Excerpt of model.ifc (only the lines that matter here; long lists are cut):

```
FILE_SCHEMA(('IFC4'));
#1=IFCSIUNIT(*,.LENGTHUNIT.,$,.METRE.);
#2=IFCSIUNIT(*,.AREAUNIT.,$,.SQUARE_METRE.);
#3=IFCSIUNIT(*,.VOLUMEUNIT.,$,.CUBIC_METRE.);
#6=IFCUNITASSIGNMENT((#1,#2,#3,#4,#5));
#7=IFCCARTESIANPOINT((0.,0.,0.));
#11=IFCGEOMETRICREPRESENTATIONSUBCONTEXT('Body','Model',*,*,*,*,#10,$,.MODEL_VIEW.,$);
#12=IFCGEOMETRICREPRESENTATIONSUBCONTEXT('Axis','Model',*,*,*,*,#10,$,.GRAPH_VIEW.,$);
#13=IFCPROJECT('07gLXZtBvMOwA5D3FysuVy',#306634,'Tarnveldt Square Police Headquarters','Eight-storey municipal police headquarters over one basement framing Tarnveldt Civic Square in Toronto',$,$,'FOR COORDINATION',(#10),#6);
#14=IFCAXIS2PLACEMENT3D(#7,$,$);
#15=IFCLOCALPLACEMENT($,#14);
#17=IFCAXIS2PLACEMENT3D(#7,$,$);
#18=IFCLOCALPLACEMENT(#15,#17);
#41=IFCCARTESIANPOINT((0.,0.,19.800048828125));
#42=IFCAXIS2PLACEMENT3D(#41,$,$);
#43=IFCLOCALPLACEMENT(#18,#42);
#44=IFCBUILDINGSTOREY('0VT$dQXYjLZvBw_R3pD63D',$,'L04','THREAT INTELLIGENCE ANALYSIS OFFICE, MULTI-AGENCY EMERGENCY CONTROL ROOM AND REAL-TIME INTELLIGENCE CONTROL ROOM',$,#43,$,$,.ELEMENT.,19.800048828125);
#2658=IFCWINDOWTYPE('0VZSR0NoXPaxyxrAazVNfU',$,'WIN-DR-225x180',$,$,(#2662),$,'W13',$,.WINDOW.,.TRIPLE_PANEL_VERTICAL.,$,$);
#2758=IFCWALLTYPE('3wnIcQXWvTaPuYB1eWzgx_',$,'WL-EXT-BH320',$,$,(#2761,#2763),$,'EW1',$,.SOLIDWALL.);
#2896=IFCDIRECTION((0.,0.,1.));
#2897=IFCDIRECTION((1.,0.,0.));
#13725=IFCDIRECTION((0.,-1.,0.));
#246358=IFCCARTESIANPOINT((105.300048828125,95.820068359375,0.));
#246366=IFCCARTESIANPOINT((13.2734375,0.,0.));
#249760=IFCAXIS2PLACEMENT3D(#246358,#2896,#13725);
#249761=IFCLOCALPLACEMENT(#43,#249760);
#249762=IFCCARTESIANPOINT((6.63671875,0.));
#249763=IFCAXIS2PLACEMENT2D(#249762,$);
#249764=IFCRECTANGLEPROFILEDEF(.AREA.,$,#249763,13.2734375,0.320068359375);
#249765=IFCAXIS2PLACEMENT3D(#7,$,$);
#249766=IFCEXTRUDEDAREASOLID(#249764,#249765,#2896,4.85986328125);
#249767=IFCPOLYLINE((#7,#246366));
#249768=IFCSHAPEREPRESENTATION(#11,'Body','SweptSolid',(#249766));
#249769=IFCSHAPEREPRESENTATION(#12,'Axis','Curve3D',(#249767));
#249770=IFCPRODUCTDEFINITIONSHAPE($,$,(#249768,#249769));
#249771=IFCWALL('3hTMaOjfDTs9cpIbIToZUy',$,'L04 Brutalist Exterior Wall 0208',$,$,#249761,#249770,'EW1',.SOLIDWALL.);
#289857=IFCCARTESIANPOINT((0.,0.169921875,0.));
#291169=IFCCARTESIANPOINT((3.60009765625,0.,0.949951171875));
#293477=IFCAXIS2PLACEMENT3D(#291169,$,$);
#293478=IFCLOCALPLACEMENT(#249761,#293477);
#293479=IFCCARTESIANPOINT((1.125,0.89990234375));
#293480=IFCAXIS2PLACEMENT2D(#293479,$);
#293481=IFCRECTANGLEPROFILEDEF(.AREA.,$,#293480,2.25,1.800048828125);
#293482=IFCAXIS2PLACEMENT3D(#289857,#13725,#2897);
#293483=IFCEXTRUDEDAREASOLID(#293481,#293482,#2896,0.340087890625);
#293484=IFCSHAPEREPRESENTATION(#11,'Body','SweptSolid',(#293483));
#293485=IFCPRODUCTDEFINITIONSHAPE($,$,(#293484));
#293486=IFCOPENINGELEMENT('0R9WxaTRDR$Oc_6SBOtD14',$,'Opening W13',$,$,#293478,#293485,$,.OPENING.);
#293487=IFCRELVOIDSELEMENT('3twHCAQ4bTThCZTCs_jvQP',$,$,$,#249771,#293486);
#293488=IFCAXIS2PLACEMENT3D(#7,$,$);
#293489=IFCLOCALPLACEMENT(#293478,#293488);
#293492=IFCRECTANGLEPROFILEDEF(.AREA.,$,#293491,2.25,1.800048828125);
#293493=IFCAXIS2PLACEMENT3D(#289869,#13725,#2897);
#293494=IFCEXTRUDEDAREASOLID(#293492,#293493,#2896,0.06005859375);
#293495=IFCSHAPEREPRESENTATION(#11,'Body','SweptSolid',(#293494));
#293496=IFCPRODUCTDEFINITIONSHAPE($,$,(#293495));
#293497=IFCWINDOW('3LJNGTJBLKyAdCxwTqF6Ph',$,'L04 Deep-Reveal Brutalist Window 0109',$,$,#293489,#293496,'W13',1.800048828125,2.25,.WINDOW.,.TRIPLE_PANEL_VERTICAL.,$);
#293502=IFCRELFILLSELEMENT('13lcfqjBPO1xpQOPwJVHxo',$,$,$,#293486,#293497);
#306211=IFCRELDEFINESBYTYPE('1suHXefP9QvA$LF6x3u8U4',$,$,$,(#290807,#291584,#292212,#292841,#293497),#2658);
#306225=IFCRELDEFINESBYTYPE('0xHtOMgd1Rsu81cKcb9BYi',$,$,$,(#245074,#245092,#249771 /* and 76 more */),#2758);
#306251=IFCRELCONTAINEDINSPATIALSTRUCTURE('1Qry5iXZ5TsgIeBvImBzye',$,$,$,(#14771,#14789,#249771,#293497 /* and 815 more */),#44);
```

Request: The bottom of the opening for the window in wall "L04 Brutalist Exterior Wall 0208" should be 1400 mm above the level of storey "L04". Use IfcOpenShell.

```python
import numpy as np
import ifcopenshell
import ifcopenshell.api.geometry
import ifcopenshell.geom
import ifcopenshell.util.element
import ifcopenshell.util.placement
import ifcopenshell.util.shape
import ifcopenshell.util.unit

model = ifcopenshell.open("model.ifc")
unit_scale = ifcopenshell.util.unit.calculate_unit_scale(model)

window = model.by_id(293497)
opening = window.FillsVoids[0].RelatingOpeningElement
storey = ifcopenshell.util.element.get_container(window, ifc_class="IfcBuildingStorey")
level = ifcopenshell.util.placement.get_local_placement(storey.ObjectPlacement)[2, 3]

# The opening's origin need not be at the sill, so measure its lowest point.
shape = ifcopenshell.geom.create_shape(ifcopenshell.geom.settings(), opening)
bottom = ifcopenshell.util.shape.get_shape_bottom_elevation(shape, shape.geometry) / unit_scale
dz = level + 1.4 / unit_scale - bottom

shift = np.array([0.0, 0.0, dz])
# The window is placed relative to its opening, so it follows when the opening moves.
matrix = ifcopenshell.util.placement.get_local_placement(opening.ObjectPlacement)
matrix[:3, 3] += shift
ifcopenshell.api.geometry.edit_object_placement(
    model, product=opening, matrix=matrix, is_si=False, should_transform_children=True
)

print(f"moved by {dz * unit_scale:+.3f} m")

model.write("model_updated.ifc")
```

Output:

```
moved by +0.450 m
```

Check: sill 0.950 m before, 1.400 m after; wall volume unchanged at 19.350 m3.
